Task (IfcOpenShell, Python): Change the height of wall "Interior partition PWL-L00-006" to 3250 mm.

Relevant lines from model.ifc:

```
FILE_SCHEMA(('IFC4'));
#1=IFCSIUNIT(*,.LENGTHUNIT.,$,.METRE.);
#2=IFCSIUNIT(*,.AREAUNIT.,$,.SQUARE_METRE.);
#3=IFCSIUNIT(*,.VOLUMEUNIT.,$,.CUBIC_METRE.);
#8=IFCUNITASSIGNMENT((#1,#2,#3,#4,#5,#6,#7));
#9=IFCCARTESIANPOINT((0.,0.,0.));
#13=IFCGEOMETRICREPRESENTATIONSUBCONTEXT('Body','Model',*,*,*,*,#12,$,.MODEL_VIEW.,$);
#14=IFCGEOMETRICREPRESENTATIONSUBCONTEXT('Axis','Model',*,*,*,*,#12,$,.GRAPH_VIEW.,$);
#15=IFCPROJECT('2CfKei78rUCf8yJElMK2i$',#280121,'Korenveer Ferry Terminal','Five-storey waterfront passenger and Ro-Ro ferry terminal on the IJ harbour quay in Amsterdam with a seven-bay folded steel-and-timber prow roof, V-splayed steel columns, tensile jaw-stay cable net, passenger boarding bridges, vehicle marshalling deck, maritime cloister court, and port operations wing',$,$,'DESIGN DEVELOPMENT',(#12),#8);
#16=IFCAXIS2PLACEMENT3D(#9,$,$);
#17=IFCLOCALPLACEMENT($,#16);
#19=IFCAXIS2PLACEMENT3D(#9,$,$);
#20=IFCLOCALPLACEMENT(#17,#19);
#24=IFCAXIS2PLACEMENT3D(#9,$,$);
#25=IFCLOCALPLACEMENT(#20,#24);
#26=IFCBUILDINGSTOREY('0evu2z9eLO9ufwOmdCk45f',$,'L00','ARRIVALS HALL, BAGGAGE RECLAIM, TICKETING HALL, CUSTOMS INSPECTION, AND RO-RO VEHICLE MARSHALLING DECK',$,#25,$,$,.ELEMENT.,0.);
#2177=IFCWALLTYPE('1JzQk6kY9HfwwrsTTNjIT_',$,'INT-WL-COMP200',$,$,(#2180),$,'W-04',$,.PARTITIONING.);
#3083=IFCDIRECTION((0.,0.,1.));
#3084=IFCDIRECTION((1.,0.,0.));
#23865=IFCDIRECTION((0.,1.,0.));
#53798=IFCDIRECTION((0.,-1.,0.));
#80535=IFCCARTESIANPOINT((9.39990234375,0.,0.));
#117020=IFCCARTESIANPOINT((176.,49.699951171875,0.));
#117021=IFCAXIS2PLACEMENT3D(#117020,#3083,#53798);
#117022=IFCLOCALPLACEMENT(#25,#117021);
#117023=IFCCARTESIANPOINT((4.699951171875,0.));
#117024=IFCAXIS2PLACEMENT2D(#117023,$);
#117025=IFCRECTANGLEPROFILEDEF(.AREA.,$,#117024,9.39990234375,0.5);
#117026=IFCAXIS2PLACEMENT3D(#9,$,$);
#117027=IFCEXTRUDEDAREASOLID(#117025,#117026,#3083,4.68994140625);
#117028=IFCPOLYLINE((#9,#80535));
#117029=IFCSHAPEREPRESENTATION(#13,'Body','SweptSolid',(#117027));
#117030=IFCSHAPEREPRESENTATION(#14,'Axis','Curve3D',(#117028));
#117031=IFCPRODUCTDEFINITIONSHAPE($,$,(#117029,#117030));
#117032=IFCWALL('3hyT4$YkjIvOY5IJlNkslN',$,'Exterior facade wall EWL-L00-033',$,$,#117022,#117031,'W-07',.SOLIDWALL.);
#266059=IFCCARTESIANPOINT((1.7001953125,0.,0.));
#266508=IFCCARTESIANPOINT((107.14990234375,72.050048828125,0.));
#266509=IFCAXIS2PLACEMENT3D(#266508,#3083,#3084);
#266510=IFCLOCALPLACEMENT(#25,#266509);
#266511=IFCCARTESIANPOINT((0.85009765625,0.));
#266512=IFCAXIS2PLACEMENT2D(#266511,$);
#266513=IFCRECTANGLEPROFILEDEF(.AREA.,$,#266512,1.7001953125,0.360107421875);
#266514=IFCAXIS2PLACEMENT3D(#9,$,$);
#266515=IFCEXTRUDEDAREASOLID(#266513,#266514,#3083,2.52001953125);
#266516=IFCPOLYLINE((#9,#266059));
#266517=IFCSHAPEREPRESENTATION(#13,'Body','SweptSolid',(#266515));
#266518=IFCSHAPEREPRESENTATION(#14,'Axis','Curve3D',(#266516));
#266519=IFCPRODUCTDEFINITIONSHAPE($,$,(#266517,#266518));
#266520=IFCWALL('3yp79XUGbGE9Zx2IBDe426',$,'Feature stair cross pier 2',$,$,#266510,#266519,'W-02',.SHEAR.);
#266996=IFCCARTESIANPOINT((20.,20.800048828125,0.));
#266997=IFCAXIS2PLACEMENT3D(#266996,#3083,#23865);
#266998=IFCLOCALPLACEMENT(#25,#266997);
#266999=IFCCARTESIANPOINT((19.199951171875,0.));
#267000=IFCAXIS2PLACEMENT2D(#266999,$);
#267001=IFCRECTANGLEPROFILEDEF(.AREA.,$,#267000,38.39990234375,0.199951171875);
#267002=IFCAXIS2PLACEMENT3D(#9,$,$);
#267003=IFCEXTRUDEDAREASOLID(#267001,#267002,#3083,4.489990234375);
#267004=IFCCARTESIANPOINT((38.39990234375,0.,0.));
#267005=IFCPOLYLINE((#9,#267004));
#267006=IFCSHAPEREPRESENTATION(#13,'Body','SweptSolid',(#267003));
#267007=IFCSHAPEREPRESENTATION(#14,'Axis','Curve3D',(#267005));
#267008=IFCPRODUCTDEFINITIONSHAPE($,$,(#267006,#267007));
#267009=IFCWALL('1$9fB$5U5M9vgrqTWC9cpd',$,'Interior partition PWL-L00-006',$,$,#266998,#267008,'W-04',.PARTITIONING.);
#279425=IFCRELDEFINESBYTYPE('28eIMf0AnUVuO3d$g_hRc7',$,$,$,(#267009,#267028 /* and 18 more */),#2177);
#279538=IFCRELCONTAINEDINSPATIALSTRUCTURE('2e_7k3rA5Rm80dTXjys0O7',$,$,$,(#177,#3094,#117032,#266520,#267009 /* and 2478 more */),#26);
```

```python
import ifcopenshell
import ifcopenshell.geom
import ifcopenshell.util.representation
import ifcopenshell.util.shape
import ifcopenshell.util.unit

model = ifcopenshell.open("model.ifc")
unit_scale = ifcopenshell.util.unit.calculate_unit_scale(model)
settings = ifcopenshell.geom.settings()


def volume(element):
    """Net volume in cubic metres, openings subtracted."""
    shape = ifcopenshell.geom.create_shape(settings, element)
    return ifcopenshell.util.shape.get_volume(shape.geometry)


wall = model.by_id(267009)
before = volume(wall)

body = ifcopenshell.util.representation.get_representation(wall, "Model", "Body")
solid = body.Items[0]
old_height = solid.Depth
solid.Depth = 3.25 / unit_scale
after = volume(wall)

print(f"height {old_height:g} -> {solid.Depth:g}, volume {before:.3f} -> {after:.3f} m3")

model.write("model_v2.ifc")
```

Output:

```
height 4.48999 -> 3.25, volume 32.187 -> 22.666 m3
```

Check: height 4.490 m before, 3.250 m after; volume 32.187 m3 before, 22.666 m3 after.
